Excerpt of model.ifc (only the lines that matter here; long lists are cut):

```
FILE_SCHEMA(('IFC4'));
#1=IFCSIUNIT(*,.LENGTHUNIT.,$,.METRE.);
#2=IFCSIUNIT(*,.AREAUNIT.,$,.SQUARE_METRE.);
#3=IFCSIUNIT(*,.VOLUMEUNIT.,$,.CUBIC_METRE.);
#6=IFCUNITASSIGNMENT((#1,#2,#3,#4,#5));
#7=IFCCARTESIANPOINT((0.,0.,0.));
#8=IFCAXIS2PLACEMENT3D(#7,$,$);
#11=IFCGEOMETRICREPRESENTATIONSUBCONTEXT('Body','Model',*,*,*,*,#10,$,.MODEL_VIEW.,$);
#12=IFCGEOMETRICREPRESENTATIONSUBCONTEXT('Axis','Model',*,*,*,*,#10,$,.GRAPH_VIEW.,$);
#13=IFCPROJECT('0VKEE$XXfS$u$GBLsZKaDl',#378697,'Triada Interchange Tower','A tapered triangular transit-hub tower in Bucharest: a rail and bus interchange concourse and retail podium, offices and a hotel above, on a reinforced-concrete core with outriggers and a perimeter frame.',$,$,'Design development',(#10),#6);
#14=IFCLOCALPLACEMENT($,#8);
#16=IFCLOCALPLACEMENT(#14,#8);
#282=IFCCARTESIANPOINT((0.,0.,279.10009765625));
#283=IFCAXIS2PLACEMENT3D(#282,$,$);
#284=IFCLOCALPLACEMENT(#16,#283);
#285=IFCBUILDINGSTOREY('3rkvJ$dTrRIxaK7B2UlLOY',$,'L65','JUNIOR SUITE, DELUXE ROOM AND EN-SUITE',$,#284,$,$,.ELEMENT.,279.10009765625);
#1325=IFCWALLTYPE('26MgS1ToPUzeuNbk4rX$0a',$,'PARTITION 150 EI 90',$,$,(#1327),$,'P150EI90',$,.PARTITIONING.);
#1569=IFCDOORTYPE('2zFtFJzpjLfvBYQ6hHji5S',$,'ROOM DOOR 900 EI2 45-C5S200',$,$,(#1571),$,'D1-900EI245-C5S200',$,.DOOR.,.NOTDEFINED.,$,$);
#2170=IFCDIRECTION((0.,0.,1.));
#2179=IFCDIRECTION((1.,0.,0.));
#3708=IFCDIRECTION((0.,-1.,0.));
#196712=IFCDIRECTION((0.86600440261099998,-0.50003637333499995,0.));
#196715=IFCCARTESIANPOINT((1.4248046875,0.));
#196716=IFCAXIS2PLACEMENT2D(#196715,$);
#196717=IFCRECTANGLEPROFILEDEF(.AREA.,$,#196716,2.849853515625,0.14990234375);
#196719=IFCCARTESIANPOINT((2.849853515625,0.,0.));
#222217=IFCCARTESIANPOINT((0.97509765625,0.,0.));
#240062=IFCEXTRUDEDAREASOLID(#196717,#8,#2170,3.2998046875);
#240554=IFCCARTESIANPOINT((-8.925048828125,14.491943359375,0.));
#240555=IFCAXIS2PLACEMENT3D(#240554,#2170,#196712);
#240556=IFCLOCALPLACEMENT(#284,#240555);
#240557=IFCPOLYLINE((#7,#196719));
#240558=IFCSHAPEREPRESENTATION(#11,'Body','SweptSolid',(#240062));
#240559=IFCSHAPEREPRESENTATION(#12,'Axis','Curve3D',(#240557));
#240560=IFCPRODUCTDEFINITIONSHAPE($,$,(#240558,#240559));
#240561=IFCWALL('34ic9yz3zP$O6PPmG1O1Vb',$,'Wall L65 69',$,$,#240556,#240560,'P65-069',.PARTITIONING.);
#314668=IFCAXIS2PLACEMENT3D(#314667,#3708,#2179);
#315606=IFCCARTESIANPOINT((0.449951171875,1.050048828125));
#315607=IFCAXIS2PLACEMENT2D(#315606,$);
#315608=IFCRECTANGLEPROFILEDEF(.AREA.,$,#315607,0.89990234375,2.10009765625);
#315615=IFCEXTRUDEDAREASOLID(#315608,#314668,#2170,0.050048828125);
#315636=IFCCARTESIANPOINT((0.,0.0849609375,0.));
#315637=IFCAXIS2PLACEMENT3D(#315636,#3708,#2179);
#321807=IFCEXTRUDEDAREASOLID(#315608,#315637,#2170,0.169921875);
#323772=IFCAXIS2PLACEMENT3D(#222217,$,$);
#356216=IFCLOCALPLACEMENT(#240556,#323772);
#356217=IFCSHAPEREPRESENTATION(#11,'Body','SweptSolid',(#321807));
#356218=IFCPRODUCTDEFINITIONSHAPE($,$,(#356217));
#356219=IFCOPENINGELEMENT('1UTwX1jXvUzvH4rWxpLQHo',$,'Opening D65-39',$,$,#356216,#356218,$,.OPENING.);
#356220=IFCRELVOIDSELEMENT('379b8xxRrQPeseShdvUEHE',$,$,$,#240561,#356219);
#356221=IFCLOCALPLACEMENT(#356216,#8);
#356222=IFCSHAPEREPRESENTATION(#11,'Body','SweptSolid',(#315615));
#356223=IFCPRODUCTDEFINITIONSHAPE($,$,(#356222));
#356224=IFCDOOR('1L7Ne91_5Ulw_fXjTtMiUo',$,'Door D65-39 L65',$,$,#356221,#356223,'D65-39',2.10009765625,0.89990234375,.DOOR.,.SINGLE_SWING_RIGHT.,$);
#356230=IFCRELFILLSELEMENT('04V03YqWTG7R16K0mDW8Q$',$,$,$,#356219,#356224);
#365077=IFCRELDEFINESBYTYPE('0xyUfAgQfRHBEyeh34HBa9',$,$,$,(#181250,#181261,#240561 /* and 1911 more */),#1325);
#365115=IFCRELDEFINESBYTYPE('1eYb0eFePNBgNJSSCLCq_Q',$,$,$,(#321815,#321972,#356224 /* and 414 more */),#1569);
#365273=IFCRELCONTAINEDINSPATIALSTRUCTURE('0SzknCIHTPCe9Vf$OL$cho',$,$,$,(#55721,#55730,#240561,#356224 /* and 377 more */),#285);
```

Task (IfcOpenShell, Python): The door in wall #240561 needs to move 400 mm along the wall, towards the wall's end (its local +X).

```python
import ifcopenshell
import ifcopenshell.api.geometry
import ifcopenshell.util.placement

model = ifcopenshell.open("model.ifc")

door = model.by_id(356224)
opening = door.FillsVoids[0].RelatingOpeningElement
wall = opening.VoidsElements[0].RelatingBuildingElement

wall_matrix = ifcopenshell.util.placement.get_local_placement(wall.ObjectPlacement)
shift = wall_matrix[:3, 0] * 0.4
before = ifcopenshell.util.placement.get_local_placement(door.ObjectPlacement)[:3, 3].copy()

# The door is placed relative to its opening, so it follows when the opening moves.
matrix = ifcopenshell.util.placement.get_local_placement(opening.ObjectPlacement)
matrix[:3, 3] += shift
ifcopenshell.api.geometry.edit_object_placement(
    model, product=opening, matrix=matrix, is_si=False, should_transform_children=True
)

after = ifcopenshell.util.placement.get_local_placement(door.ObjectPlacement)[:3, 3]
print("door moved by", (after - before).round(3) + 0.0)

model.write("model_updated.ifc")
```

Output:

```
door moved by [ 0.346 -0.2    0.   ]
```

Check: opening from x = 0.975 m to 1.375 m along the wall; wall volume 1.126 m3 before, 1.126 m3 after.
